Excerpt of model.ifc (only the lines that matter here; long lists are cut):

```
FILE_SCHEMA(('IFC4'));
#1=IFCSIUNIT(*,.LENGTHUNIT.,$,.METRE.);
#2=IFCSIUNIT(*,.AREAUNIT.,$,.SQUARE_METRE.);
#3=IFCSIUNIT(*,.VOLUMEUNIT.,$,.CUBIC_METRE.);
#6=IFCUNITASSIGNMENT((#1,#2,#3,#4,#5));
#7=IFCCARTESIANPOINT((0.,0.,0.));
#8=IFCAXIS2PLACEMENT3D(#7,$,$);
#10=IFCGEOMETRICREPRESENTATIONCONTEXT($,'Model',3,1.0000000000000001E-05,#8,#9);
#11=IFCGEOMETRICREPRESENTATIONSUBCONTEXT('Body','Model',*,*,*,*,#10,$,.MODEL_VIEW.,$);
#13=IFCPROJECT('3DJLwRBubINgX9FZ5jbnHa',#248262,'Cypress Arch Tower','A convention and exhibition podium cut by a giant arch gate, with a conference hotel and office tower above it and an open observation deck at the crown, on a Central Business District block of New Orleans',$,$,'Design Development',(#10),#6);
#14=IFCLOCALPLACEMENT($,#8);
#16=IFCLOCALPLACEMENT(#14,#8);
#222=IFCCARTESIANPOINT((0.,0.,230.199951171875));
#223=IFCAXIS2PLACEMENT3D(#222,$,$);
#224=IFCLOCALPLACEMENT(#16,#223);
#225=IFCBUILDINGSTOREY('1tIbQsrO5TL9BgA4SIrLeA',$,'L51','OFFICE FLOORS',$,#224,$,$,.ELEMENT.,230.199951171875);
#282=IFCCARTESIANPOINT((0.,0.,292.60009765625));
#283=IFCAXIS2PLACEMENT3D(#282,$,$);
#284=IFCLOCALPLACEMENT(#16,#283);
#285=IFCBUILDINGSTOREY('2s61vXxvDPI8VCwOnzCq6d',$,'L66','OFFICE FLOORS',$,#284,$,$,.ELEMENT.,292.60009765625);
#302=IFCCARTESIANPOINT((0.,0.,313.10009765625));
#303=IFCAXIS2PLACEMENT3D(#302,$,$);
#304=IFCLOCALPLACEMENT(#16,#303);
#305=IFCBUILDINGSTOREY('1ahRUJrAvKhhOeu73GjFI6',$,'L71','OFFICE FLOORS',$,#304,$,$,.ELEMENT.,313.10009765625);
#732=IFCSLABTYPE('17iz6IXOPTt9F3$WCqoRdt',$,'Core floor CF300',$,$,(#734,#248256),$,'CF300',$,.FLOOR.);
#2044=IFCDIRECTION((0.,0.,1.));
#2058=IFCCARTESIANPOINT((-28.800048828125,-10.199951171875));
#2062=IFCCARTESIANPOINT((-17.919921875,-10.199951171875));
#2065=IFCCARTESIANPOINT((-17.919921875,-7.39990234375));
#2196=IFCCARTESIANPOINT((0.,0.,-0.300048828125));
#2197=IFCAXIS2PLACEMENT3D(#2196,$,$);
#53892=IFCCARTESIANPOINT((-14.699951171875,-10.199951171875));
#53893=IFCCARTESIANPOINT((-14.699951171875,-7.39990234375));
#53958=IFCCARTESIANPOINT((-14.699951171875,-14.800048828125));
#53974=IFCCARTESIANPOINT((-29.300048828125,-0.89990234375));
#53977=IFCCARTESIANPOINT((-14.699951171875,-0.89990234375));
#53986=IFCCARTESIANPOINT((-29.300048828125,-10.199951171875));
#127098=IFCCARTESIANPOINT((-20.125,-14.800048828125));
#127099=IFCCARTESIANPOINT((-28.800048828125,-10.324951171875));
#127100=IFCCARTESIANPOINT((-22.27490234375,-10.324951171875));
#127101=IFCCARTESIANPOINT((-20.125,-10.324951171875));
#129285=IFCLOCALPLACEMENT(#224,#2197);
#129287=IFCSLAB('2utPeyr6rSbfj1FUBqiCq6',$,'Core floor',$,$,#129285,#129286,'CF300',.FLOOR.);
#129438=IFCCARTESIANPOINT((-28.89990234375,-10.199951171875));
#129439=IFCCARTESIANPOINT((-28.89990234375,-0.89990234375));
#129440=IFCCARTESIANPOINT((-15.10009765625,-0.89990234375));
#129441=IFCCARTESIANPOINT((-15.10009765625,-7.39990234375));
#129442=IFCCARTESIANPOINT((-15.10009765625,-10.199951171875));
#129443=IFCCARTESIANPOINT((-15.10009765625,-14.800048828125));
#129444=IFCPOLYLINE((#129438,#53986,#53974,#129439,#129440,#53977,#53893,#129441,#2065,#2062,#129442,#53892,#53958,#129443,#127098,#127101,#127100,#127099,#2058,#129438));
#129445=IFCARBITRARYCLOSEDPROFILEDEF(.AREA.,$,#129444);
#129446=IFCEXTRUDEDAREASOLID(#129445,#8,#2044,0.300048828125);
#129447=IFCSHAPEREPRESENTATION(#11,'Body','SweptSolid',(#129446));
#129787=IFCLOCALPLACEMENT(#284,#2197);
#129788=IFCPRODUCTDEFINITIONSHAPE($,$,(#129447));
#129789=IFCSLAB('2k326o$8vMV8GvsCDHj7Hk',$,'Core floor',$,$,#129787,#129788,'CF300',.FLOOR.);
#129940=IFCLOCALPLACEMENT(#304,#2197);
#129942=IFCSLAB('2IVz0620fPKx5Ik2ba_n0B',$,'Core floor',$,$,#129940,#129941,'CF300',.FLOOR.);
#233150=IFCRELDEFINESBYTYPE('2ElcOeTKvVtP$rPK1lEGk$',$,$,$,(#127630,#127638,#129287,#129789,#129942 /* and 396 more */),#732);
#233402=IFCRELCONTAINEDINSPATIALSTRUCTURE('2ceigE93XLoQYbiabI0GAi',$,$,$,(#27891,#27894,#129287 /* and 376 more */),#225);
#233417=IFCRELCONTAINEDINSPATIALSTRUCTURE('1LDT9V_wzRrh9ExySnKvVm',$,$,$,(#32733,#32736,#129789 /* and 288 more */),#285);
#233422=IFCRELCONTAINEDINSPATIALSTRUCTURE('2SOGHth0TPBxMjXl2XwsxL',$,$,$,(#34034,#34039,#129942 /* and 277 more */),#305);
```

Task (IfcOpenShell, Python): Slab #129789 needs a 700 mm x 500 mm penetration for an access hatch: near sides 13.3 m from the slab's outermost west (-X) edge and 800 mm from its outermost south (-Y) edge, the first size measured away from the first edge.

```python
import numpy as np
import ifcopenshell
import ifcopenshell.api.feature
import ifcopenshell.api.geometry
import ifcopenshell.api.root
import ifcopenshell.geom
import ifcopenshell.util.placement
import ifcopenshell.util.representation
import ifcopenshell.util.shape
import ifcopenshell.util.unit

model = ifcopenshell.open("model.ifc")
unit_scale = ifcopenshell.util.unit.calculate_unit_scale(model)
settings = ifcopenshell.geom.settings()


def volume(element):
    """Net volume in cubic metres, openings subtracted."""
    shape = ifcopenshell.geom.create_shape(settings, element)
    return ifcopenshell.util.shape.get_volume(shape.geometry)


slab = model.by_guid("2k326o$8vMV8GvsCDHj7Hk")
before = volume(slab)

# Extent in the slab's own axes, in metres. The edges named are its -X and -Y sides.
slab_shape = ifcopenshell.geom.create_shape(settings, slab)
vertices = ifcopenshell.util.shape.get_vertices(slab_shape.geometry)
x_min, y_min, bottom = vertices.min(axis=0)
top = vertices[:, 2].max()

opening = ifcopenshell.api.root.create_entity(model, ifc_class="IfcOpeningElement", name="Access hatch opening", predefined_type="OPENING")
context = ifcopenshell.util.representation.get_context(model, "Model", "Body", "MODEL_VIEW")
width, depth = 0.7, 0.5
outline = [(0.0, 0.0), (width, 0.0), (width, depth), (0.0, depth), (0.0, 0.0)]
# Overshoot both faces by 50 mm so the cut is clean.
shape = ifcopenshell.api.geometry.add_slab_representation(
    model, context=context, depth=top - bottom + 0.1, polyline=outline
)
ifcopenshell.api.geometry.assign_representation(model, product=opening, representation=shape)

matrix = ifcopenshell.util.placement.get_local_placement(slab.ObjectPlacement)
matrix[:, 3] = matrix @ np.append(np.array([x_min + 13.3, y_min + 0.8, bottom - 0.05]) / unit_scale, 1.0)
ifcopenshell.api.geometry.edit_object_placement(model, product=opening, matrix=matrix, is_si=False)
ifcopenshell.api.feature.add_feature(model, feature=opening, element=slab)

after = volume(slab)

print(f"slab volume {before:.3f} -> {after:.3f} m3")

model.write("model_v2.ifc")
```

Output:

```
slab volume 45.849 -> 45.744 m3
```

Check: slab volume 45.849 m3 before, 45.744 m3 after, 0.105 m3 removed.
